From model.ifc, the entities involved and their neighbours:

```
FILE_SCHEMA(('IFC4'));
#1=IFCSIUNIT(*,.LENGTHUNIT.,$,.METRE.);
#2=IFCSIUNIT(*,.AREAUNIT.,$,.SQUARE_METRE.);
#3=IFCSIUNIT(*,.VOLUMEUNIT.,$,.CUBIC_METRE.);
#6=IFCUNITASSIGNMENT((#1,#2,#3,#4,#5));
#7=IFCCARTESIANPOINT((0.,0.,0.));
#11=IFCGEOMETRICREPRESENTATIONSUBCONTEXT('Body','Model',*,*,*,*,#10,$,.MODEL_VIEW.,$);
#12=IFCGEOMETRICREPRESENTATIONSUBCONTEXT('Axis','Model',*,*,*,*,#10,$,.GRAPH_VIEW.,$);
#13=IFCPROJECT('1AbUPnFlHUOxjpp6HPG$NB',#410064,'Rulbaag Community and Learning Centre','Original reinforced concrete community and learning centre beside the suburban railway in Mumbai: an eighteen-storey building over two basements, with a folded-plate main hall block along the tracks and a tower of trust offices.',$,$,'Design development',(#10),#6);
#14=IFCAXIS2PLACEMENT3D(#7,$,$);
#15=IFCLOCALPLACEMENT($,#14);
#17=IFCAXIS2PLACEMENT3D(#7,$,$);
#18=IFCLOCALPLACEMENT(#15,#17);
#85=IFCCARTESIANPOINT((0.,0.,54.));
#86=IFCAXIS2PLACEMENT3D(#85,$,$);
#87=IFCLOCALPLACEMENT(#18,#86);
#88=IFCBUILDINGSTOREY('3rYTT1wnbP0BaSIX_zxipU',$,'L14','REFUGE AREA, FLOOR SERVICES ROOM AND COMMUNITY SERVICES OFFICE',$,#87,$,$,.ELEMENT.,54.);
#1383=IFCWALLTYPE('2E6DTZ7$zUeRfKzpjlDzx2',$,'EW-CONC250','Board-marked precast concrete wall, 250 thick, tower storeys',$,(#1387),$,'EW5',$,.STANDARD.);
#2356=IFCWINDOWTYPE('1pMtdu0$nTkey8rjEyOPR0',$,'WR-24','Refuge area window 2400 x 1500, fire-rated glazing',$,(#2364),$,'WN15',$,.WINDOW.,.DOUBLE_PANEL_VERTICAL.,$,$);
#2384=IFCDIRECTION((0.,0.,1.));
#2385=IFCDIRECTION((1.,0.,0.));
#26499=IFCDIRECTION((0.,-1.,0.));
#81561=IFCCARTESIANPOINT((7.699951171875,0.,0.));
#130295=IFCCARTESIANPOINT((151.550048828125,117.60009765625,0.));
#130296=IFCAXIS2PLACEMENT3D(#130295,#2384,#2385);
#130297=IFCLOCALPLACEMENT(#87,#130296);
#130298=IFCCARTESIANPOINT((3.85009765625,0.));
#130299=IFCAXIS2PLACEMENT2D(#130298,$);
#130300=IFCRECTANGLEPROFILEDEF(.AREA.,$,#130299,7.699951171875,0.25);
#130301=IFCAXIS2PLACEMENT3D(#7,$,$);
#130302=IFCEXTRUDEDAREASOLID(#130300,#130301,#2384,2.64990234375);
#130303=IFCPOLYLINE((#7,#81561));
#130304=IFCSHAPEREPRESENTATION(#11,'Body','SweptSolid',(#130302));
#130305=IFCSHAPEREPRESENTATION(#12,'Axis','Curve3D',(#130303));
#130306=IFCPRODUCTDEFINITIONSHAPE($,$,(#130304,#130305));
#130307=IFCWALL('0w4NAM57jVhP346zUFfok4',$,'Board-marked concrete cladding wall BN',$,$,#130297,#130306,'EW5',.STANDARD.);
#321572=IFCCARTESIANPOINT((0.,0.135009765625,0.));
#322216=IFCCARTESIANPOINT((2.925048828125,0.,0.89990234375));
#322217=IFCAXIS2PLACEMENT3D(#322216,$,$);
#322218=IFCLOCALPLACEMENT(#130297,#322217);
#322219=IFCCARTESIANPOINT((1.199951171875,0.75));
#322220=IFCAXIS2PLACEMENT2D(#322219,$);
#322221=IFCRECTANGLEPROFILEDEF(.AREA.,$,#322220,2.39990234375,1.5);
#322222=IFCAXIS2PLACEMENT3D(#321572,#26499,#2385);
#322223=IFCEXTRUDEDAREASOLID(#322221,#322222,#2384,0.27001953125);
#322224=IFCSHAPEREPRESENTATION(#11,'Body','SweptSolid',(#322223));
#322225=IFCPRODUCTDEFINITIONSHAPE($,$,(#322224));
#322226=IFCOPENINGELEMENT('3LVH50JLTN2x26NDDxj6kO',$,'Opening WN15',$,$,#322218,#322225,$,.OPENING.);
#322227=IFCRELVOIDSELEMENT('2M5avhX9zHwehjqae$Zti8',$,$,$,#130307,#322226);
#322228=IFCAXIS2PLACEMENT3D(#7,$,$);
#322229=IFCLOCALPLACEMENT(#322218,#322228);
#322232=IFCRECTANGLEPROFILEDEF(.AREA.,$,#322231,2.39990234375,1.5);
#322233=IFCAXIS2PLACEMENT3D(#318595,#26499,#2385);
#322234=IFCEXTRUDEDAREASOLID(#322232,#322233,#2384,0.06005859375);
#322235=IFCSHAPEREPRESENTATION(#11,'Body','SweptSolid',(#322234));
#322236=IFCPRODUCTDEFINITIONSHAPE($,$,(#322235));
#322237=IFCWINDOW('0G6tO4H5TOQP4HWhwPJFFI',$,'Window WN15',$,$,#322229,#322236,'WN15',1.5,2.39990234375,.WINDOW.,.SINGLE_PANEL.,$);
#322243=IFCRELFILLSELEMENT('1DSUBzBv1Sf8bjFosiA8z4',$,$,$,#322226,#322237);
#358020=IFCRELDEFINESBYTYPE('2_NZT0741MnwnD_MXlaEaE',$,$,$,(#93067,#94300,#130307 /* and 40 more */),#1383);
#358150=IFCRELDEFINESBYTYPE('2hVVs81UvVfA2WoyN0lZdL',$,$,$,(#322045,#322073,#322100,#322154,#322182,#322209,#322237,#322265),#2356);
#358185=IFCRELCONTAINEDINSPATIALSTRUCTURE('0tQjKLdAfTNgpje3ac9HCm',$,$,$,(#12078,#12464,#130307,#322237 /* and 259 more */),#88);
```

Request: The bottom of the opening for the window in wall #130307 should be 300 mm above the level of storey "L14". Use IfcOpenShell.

```python
import numpy as np
import ifcopenshell
import ifcopenshell.api.geometry
import ifcopenshell.geom
import ifcopenshell.util.element
import ifcopenshell.util.placement
import ifcopenshell.util.shape
import ifcopenshell.util.unit

model = ifcopenshell.open("model.ifc")
unit_scale = ifcopenshell.util.unit.calculate_unit_scale(model)

window = model.by_id(322237)
opening = window.FillsVoids[0].RelatingOpeningElement
storey = ifcopenshell.util.element.get_container(window, ifc_class="IfcBuildingStorey")
level = ifcopenshell.util.placement.get_local_placement(storey.ObjectPlacement)[2, 3]

# The opening's origin need not be at the sill, so measure its lowest point.
shape = ifcopenshell.geom.create_shape(ifcopenshell.geom.settings(), opening)
bottom = ifcopenshell.util.shape.get_shape_bottom_elevation(shape, shape.geometry) / unit_scale
dz = level + 0.3 - bottom

shift = np.array([0.0, 0.0, dz])
# The window is placed relative to its opening, so it follows when the opening moves.
matrix = ifcopenshell.util.placement.get_local_placement(opening.ObjectPlacement)
matrix[:3, 3] += shift
ifcopenshell.api.geometry.edit_object_placement(
    model, product=opening, matrix=matrix, is_si=False, should_transform_children=True
)

print(f"moved by {dz * unit_scale:+.3f} m")

model.write("model_rev.ifc")
```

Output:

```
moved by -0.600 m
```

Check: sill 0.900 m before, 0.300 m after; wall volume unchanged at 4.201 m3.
